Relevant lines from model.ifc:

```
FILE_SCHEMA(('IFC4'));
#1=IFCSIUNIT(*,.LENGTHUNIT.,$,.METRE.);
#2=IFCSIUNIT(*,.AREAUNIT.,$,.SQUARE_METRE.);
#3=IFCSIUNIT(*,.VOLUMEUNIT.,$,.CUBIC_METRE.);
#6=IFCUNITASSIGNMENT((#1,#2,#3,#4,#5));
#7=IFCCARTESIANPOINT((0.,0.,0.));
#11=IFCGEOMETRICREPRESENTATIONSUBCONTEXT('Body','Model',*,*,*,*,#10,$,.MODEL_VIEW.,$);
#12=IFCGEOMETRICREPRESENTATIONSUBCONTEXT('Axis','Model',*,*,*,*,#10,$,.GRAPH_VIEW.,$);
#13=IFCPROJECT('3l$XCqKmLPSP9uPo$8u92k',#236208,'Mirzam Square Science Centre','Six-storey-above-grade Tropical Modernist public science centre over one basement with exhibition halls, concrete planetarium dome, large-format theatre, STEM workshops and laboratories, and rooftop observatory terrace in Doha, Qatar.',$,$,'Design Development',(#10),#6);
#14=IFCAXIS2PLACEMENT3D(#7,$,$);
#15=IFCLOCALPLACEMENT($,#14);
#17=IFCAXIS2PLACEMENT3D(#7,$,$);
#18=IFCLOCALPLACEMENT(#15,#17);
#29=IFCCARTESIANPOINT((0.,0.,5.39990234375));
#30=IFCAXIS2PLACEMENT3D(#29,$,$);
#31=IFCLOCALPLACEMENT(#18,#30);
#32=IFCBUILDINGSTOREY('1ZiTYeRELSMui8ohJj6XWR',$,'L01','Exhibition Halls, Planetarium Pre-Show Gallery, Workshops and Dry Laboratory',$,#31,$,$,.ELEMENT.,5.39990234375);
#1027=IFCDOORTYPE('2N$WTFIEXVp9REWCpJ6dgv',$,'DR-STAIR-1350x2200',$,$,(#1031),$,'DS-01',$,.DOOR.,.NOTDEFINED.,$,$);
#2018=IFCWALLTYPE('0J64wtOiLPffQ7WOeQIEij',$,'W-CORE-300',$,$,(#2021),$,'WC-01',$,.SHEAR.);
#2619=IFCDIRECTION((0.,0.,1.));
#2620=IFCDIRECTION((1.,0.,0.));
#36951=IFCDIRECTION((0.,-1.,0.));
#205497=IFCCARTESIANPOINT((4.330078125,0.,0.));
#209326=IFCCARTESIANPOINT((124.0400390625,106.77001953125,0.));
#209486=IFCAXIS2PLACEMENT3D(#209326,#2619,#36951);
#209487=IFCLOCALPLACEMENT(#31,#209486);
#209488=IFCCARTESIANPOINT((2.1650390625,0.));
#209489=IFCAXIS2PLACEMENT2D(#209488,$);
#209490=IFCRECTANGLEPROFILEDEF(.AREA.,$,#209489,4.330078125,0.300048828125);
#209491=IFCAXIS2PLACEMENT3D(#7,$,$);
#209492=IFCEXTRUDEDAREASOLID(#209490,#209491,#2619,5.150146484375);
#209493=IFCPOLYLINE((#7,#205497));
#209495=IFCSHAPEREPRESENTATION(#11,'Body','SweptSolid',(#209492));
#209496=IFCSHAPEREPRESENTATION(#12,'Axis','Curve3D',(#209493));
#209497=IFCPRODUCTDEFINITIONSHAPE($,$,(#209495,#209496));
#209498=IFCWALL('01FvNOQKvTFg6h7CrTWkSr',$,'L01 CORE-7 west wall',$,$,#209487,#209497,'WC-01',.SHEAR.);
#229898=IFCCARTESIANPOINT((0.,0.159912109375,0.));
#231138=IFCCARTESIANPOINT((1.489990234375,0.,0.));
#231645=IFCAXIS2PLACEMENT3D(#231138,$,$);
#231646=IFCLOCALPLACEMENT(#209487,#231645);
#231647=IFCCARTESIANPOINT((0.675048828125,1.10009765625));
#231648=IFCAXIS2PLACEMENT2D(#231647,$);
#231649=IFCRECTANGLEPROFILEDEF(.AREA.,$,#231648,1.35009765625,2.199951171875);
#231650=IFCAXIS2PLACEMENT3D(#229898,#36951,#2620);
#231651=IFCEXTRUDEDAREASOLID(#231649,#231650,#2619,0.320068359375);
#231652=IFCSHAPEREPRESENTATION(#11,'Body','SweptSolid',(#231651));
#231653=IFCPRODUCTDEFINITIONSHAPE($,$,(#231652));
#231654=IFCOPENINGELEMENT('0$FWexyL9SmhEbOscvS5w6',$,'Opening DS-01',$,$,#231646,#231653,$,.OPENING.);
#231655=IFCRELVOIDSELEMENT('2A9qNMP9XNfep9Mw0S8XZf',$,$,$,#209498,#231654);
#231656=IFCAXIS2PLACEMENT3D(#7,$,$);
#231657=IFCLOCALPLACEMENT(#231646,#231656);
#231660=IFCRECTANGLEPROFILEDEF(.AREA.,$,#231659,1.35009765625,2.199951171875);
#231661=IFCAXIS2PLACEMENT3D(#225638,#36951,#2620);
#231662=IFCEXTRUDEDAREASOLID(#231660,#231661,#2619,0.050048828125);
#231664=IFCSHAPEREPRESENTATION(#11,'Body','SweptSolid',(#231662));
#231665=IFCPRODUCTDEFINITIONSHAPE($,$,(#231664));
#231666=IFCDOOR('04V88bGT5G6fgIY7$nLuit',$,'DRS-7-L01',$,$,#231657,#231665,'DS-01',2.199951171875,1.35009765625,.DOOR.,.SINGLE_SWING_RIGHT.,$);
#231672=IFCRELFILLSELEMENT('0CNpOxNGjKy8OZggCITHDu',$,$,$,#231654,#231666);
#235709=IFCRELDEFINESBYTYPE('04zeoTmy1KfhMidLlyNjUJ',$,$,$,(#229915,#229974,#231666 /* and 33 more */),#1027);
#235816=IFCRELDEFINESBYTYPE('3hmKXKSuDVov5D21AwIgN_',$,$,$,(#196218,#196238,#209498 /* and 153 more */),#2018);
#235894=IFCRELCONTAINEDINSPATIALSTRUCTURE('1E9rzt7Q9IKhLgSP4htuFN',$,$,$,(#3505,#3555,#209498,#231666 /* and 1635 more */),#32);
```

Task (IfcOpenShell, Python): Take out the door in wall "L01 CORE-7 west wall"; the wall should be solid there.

```python
import ifcopenshell
import ifcopenshell.api.feature
import ifcopenshell.api.root
import ifcopenshell.geom
import ifcopenshell.util.shape

model = ifcopenshell.open("model.ifc")
settings = ifcopenshell.geom.settings()


def volume(element):
    """Net volume in cubic metres, openings subtracted."""
    shape = ifcopenshell.geom.create_shape(settings, element)
    return ifcopenshell.util.shape.get_volume(shape.geometry)


door = model.by_guid("04V88bGT5G6fgIY7$nLuit")
opening = door.FillsVoids[0].RelatingOpeningElement
wall = opening.VoidsElements[0].RelatingBuildingElement
before = volume(wall)

ifcopenshell.api.root.remove_product(model, product=door)
ifcopenshell.api.feature.remove_feature(model, feature=opening)

after = volume(wall)

print(f"wall volume {before:.3f} -> {after:.3f} m3")

model.write("model_v2.ifc")
```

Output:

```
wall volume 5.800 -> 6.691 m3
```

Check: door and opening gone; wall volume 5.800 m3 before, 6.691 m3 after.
